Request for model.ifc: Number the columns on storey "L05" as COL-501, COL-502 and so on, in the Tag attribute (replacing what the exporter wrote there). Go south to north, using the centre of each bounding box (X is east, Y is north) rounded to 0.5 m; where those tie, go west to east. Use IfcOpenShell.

First a look at what the model holds.

```python
import ifcopenshell
import ifcopenshell.util.element
import ifcopenshell.util.placement

model = ifcopenshell.open("model.ifc")
print(model.schema)
storey = next(s for s in model.by_type("IfcBuildingStorey") if s.Name == "L05")
columns = [e for e in ifcopenshell.util.element.get_decomposition(storey) if e.is_a("IfcColumn")]
for e in sorted(columns, key=lambda e: e.id()):
    origin = ifcopenshell.util.placement.get_local_placement(e.ObjectPlacement)[:3, 3]
    print(e.id(), e.Tag, e.Name, origin.round(2) + 0.0, sep=" | ")
```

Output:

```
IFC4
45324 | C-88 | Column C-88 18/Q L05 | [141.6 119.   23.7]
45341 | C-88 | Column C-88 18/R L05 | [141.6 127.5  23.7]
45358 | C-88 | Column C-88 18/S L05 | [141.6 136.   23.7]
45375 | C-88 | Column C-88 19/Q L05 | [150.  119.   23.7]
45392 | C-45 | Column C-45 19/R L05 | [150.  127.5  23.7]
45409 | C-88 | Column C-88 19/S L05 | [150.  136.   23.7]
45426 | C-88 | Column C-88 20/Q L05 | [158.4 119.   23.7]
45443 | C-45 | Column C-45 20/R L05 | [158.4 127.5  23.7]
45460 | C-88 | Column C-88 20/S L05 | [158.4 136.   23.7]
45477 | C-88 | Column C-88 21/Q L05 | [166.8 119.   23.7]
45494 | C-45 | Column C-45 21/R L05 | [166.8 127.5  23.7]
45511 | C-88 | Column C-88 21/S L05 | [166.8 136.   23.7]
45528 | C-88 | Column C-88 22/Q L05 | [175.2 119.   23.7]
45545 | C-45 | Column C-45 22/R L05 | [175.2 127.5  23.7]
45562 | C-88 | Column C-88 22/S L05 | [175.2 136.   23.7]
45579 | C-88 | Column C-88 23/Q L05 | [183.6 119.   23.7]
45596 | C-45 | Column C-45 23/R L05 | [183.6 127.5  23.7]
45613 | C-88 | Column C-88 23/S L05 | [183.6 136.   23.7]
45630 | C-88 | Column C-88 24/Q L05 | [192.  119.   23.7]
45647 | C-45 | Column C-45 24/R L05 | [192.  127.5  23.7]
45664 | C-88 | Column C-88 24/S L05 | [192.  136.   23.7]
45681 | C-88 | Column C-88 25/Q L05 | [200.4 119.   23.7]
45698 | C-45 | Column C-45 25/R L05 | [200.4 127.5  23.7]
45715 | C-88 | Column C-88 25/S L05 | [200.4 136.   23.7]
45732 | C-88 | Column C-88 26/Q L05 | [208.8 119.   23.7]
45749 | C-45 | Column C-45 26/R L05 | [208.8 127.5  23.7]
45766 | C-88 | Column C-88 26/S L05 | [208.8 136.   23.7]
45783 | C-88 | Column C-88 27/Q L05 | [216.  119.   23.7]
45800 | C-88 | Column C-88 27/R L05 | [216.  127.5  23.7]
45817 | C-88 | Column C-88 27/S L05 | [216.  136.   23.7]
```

```python
import ifcopenshell
import ifcopenshell.geom
import ifcopenshell.util.element
import ifcopenshell.util.shape

model = ifcopenshell.open("model.ifc")
settings = ifcopenshell.geom.settings()
settings.set("use-world-coords", True)


def centre(element):
    shape = ifcopenshell.geom.create_shape(settings, element)
    return ifcopenshell.util.shape.get_bbox_centroid(shape.geometry)


storey = next(s for s in model.by_type("IfcBuildingStorey") if s.Name == "L05")
columns = [e for e in ifcopenshell.util.element.get_decomposition(storey) if e.is_a("IfcColumn")]

# Insertion points can sit at a corner or the storey origin, so sort by the geometry (in metres).
centres = {e: centre(e) for e in columns}
columns.sort(key=lambda e: (round(centres[e][1] / 0.5), centres[e][0]))

for i, e in enumerate(columns, start=1):
    number = f"COL-5{i:02d}"
    e.Tag = number
    print(e.id(), number)

model.write("model_rev.ifc")
```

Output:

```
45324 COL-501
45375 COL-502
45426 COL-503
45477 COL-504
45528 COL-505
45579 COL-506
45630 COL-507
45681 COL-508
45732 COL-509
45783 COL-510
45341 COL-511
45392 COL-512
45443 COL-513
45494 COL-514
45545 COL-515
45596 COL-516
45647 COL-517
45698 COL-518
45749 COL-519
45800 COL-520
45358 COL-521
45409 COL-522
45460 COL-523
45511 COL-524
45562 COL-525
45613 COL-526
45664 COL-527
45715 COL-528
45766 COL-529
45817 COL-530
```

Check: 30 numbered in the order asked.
